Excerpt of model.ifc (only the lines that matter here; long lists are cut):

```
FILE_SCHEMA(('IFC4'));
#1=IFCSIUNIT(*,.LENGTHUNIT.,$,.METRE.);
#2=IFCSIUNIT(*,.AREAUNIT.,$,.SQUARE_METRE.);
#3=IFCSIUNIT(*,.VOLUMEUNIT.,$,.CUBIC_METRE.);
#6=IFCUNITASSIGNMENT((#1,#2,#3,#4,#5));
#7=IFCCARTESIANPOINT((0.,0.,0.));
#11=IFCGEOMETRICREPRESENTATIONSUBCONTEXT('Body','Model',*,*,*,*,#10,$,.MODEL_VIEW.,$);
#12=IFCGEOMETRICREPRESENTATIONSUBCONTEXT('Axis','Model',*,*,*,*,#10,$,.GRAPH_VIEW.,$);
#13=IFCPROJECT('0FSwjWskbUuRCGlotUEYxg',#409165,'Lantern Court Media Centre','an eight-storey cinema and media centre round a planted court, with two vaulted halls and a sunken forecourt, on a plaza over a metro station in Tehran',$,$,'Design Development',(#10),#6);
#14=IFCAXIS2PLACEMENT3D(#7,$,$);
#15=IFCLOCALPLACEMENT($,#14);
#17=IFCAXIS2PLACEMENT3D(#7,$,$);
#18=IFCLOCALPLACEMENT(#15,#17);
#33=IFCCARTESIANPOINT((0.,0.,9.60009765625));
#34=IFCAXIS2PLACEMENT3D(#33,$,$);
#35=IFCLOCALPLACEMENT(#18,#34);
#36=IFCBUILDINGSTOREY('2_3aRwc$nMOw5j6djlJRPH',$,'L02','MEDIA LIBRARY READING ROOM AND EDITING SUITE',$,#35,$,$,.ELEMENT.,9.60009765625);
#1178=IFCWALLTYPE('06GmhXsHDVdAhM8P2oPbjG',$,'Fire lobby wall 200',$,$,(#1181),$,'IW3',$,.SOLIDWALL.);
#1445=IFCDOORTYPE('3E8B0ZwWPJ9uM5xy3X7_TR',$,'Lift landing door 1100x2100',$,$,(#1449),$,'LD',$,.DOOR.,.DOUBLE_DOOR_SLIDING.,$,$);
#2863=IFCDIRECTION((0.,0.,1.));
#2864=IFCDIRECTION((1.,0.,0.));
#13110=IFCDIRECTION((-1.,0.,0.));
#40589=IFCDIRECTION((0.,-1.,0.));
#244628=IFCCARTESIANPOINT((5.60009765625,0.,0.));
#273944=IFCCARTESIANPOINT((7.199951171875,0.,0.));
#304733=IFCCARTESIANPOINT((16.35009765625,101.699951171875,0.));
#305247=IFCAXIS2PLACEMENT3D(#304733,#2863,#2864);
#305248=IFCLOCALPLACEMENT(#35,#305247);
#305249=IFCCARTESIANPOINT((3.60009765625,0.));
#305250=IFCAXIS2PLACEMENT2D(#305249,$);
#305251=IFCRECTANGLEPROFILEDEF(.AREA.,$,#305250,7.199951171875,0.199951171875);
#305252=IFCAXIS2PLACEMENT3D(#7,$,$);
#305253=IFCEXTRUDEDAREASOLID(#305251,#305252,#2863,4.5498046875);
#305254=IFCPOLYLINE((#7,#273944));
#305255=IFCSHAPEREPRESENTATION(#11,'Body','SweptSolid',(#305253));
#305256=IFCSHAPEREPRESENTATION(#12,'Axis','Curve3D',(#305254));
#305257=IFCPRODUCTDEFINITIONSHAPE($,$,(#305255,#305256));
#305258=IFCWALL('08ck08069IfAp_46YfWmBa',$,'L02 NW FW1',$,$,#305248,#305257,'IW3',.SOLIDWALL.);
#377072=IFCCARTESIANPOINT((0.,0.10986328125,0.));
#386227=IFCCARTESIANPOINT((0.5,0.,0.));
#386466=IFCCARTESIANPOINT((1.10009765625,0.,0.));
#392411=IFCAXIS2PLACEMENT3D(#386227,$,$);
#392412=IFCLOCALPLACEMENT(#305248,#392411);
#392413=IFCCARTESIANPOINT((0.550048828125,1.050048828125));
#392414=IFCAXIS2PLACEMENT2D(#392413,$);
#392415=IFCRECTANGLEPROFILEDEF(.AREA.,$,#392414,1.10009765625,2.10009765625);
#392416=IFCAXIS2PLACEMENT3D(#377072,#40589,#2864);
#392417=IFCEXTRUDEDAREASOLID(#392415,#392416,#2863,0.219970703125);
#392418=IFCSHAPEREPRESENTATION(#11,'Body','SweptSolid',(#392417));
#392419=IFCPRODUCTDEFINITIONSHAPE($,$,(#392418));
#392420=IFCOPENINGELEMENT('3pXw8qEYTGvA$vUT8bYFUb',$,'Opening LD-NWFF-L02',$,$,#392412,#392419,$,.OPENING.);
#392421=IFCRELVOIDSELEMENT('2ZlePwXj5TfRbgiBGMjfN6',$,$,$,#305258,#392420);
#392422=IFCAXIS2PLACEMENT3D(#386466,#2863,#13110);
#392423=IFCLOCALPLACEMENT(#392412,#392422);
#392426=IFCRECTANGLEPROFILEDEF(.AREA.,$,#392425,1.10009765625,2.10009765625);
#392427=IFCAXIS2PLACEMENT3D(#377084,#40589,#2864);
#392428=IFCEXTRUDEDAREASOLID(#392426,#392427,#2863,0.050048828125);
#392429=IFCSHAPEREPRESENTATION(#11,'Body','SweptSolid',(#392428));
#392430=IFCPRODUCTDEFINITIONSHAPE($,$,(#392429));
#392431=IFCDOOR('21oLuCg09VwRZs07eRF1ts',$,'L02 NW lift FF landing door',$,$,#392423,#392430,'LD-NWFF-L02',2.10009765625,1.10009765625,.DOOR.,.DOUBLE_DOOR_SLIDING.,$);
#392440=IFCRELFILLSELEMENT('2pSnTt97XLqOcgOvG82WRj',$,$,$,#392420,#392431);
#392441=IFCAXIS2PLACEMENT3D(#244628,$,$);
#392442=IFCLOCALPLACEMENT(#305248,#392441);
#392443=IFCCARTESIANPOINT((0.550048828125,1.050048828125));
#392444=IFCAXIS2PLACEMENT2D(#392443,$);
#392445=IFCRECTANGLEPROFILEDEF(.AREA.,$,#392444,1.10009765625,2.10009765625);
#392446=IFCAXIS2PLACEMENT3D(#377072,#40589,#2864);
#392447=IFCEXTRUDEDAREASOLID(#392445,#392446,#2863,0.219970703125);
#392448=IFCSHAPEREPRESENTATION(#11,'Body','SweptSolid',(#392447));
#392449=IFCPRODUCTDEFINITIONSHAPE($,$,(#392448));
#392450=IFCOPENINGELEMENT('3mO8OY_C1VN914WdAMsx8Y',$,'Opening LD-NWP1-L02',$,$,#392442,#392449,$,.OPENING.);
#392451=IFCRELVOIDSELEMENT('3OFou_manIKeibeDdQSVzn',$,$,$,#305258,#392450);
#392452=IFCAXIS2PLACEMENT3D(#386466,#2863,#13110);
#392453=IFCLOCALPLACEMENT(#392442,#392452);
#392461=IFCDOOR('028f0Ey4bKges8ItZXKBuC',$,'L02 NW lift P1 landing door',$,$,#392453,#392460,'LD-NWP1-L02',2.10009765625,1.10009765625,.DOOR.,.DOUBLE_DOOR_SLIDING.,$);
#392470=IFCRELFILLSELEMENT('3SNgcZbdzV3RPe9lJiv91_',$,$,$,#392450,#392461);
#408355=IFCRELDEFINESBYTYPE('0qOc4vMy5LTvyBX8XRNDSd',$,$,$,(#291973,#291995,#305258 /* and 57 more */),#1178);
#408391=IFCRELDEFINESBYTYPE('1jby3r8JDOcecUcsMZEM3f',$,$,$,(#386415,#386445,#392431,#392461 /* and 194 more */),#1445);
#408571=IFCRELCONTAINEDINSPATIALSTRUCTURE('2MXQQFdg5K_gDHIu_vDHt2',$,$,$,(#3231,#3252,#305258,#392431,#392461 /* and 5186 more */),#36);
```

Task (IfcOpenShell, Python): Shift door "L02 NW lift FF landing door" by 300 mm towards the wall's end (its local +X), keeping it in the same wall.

```python
import ifcopenshell
import ifcopenshell.api.geometry
import ifcopenshell.util.placement

model = ifcopenshell.open("model.ifc")

door = model.by_guid("21oLuCg09VwRZs07eRF1ts")
opening = door.FillsVoids[0].RelatingOpeningElement
wall = opening.VoidsElements[0].RelatingBuildingElement

wall_matrix = ifcopenshell.util.placement.get_local_placement(wall.ObjectPlacement)
shift = wall_matrix[:3, 0] * 0.3
before = ifcopenshell.util.placement.get_local_placement(door.ObjectPlacement)[:3, 3].copy()

# The door is placed relative to its opening, so it follows when the opening moves.
matrix = ifcopenshell.util.placement.get_local_placement(opening.ObjectPlacement)
matrix[:3, 3] += shift
ifcopenshell.api.geometry.edit_object_placement(
    model, product=opening, matrix=matrix, is_si=False, should_transform_children=True
)

after = ifcopenshell.util.placement.get_local_placement(door.ObjectPlacement)[:3, 3]
print("door moved by", (after - before).round(3) + 0.0)

model.write("model_updated.ifc")
```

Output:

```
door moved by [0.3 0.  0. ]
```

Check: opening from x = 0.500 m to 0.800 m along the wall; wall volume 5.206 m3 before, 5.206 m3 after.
